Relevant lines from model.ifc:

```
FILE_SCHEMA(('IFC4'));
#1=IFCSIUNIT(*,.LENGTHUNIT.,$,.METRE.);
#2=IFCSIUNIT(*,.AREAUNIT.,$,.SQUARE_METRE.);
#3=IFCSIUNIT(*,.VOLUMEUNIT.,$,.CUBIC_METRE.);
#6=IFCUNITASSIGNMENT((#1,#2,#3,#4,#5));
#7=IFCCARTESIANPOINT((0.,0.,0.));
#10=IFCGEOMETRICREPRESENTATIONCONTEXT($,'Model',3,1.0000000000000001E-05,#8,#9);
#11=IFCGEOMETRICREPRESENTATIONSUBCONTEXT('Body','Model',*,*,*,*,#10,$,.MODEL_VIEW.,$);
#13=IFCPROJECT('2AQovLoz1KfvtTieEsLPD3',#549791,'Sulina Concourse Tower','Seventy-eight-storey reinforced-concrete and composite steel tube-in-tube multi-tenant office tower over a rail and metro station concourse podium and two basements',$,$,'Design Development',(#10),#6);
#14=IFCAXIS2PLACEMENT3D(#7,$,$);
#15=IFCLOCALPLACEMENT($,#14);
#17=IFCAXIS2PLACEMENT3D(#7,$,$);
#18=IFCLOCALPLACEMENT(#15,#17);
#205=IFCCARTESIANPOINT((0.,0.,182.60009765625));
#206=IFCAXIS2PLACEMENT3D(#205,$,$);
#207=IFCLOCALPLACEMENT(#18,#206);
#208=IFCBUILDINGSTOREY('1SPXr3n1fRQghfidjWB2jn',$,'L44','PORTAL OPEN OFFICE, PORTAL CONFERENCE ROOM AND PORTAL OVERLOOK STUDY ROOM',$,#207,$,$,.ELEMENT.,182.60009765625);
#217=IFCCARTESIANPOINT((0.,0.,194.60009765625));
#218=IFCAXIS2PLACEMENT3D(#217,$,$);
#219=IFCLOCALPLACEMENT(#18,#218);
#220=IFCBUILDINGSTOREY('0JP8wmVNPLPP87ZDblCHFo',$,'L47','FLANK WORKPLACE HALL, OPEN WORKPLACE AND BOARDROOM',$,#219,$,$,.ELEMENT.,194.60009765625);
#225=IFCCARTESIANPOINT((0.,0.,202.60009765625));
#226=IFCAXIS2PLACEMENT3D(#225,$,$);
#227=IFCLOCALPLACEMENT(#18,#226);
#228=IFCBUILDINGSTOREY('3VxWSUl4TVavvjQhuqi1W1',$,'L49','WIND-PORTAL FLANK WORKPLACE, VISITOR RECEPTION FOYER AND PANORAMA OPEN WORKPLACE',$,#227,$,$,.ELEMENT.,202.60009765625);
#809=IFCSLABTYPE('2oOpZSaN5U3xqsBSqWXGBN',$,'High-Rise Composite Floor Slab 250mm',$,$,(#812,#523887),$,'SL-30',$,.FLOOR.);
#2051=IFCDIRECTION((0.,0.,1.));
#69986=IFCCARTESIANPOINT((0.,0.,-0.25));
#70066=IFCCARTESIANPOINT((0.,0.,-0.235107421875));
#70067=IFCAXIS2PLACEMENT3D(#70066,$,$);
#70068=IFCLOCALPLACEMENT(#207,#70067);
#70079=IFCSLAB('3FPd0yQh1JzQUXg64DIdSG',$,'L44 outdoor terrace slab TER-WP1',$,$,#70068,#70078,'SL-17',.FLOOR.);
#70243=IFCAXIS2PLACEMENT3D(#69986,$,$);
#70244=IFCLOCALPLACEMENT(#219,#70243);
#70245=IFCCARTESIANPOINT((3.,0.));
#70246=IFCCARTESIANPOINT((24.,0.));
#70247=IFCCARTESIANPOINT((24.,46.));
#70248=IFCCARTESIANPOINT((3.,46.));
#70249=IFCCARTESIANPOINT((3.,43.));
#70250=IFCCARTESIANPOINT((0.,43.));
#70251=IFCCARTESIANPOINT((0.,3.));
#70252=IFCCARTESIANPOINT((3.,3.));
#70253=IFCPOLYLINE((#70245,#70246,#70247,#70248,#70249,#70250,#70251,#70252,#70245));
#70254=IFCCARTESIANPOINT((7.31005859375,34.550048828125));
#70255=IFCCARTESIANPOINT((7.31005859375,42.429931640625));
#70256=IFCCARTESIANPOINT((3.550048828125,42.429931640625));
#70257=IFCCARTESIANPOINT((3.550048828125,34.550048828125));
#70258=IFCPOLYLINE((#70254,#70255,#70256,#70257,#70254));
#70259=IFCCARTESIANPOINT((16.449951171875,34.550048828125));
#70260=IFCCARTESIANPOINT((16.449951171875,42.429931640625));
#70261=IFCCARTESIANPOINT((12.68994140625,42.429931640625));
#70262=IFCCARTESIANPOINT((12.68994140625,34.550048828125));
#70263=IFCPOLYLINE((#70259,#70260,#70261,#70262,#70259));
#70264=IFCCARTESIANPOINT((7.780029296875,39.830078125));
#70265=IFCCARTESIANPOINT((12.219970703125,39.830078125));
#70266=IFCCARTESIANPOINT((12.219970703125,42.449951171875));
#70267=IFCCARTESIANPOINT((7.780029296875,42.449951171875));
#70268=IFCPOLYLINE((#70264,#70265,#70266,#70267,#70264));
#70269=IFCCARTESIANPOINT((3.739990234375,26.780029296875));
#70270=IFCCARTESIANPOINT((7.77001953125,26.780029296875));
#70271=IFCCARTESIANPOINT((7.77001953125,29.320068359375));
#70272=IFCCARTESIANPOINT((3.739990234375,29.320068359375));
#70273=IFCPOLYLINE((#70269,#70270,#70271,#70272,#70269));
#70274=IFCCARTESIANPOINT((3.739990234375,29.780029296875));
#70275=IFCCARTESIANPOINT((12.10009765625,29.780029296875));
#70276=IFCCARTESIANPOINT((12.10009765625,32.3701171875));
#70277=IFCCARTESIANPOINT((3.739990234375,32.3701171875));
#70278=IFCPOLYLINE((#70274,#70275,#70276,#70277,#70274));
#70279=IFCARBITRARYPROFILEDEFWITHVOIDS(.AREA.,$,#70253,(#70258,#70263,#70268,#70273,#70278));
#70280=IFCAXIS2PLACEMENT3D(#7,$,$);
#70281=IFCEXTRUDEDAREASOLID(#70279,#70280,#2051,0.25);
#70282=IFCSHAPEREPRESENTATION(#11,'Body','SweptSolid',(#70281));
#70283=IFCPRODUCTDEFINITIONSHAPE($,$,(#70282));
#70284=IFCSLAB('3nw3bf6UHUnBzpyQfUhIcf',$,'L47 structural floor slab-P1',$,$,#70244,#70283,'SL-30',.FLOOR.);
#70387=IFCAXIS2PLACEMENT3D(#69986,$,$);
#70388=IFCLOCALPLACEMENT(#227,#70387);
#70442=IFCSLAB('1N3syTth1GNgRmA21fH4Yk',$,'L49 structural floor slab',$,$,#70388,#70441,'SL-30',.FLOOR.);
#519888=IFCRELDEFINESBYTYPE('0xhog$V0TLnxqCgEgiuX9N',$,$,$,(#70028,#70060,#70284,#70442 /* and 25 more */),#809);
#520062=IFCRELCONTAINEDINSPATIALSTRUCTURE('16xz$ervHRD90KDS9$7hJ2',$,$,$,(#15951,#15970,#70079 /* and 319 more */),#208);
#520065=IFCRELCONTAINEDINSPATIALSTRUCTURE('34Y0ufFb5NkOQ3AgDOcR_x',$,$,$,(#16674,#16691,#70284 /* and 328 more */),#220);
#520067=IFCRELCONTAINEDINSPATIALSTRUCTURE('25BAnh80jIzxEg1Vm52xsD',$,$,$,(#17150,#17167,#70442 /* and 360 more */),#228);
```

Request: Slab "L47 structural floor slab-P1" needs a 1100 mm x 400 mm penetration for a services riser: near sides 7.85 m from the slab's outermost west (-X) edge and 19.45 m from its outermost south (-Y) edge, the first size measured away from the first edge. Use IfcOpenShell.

```python
import numpy as np
import ifcopenshell
import ifcopenshell.api.feature
import ifcopenshell.api.geometry
import ifcopenshell.api.root
import ifcopenshell.geom
import ifcopenshell.util.placement
import ifcopenshell.util.representation
import ifcopenshell.util.shape
import ifcopenshell.util.unit

model = ifcopenshell.open("model.ifc")
unit_scale = ifcopenshell.util.unit.calculate_unit_scale(model)
settings = ifcopenshell.geom.settings()


def volume(element):
    """Net volume in cubic metres, openings subtracted."""
    shape = ifcopenshell.geom.create_shape(settings, element)
    return ifcopenshell.util.shape.get_volume(shape.geometry)


slab = model.by_guid("3nw3bf6UHUnBzpyQfUhIcf")
before = volume(slab)

# Extent in the slab's own axes, in metres. The edges named are its -X and -Y sides.
slab_shape = ifcopenshell.geom.create_shape(settings, slab)
vertices = ifcopenshell.util.shape.get_vertices(slab_shape.geometry)
x_min, y_min, bottom = vertices.min(axis=0)
top = vertices[:, 2].max()

opening = ifcopenshell.api.root.create_entity(model, ifc_class="IfcOpeningElement", name="Services riser opening", predefined_type="OPENING")
context = ifcopenshell.util.representation.get_context(model, "Model", "Body", "MODEL_VIEW")
width, depth = 1.1, 0.4
outline = [(0.0, 0.0), (width, 0.0), (width, depth), (0.0, depth), (0.0, 0.0)]
# Overshoot both faces by 50 mm so the cut is clean.
shape = ifcopenshell.api.geometry.add_slab_representation(
    model, context=context, depth=top - bottom + 0.1, polyline=outline
)
ifcopenshell.api.geometry.assign_representation(model, product=opening, representation=shape)

matrix = ifcopenshell.util.placement.get_local_placement(slab.ObjectPlacement)
matrix[:, 3] = matrix @ np.append(np.array([x_min + 7.85, y_min + 19.45, bottom - 0.05]) / unit_scale, 1.0)
ifcopenshell.api.geometry.edit_object_placement(model, product=opening, matrix=matrix, is_si=False)
ifcopenshell.api.feature.add_feature(model, feature=opening, element=slab)

after = volume(slab)

print(f"slab volume {before:.3f} -> {after:.3f} m3")

model.write("model_edited.ifc")
```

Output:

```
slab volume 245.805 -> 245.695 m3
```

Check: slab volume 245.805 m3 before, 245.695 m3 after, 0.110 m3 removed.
